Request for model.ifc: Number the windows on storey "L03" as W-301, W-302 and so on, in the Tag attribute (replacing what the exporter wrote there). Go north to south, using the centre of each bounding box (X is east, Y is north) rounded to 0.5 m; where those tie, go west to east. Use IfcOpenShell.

First a look at what the model holds.

```python
import ifcopenshell
import ifcopenshell.util.element
import ifcopenshell.util.placement

model = ifcopenshell.open("model.ifc")
print(model.schema)
storey = next(s for s in model.by_type("IfcBuildingStorey") if s.Name == "L03")
windows = [e for e in ifcopenshell.util.element.get_decomposition(storey) if e.is_a("IfcWindow")]
for e in sorted(windows, key=lambda e: e.id()):
    origin = ifcopenshell.util.placement.get_local_placement(e.ObjectPlacement)[:3, 3]
    print(e.id(), e.Tag, e.Name, origin.round(2) + 0.0, sep=" | ")
```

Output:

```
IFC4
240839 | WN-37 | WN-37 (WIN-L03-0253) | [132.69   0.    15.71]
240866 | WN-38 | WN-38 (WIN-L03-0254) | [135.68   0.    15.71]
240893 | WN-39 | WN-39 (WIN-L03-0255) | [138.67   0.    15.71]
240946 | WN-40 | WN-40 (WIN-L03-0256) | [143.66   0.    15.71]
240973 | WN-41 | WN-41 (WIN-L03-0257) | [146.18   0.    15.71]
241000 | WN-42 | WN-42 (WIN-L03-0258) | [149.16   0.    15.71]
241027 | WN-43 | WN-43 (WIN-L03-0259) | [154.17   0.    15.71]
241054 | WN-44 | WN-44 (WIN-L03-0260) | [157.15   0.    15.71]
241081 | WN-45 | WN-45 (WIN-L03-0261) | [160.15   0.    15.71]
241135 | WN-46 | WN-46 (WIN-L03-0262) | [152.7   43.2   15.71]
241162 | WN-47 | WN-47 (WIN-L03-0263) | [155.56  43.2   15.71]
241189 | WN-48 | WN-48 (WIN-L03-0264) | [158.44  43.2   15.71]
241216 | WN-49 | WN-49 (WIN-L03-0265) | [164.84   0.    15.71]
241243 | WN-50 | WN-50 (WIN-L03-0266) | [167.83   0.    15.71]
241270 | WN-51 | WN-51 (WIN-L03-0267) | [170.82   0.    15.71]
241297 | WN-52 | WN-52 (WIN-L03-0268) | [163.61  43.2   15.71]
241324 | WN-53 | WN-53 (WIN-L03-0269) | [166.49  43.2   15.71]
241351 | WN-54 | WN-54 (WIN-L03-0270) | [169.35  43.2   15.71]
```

```python
import ifcopenshell
import ifcopenshell.geom
import ifcopenshell.util.element
import ifcopenshell.util.shape

model = ifcopenshell.open("model.ifc")
settings = ifcopenshell.geom.settings()
settings.set("use-world-coords", True)


def centre(element):
    shape = ifcopenshell.geom.create_shape(settings, element)
    return ifcopenshell.util.shape.get_bbox_centroid(shape.geometry)


storey = next(s for s in model.by_type("IfcBuildingStorey") if s.Name == "L03")
windows = [e for e in ifcopenshell.util.element.get_decomposition(storey) if e.is_a("IfcWindow")]

# Insertion points can sit at a corner or the storey origin, so sort by the geometry (in metres).
centres = {e: centre(e) for e in windows}
windows.sort(key=lambda e: (-round(centres[e][1] / 0.5), centres[e][0]))

for i, e in enumerate(windows, start=1):
    number = f"W-3{i:02d}"
    e.Tag = number
    print(e.id(), number)

model.write("model_edited.ifc")
```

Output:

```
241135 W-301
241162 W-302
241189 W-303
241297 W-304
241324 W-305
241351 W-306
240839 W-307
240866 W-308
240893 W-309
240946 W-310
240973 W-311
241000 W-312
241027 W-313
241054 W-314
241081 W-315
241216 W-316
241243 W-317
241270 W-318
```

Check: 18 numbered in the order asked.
